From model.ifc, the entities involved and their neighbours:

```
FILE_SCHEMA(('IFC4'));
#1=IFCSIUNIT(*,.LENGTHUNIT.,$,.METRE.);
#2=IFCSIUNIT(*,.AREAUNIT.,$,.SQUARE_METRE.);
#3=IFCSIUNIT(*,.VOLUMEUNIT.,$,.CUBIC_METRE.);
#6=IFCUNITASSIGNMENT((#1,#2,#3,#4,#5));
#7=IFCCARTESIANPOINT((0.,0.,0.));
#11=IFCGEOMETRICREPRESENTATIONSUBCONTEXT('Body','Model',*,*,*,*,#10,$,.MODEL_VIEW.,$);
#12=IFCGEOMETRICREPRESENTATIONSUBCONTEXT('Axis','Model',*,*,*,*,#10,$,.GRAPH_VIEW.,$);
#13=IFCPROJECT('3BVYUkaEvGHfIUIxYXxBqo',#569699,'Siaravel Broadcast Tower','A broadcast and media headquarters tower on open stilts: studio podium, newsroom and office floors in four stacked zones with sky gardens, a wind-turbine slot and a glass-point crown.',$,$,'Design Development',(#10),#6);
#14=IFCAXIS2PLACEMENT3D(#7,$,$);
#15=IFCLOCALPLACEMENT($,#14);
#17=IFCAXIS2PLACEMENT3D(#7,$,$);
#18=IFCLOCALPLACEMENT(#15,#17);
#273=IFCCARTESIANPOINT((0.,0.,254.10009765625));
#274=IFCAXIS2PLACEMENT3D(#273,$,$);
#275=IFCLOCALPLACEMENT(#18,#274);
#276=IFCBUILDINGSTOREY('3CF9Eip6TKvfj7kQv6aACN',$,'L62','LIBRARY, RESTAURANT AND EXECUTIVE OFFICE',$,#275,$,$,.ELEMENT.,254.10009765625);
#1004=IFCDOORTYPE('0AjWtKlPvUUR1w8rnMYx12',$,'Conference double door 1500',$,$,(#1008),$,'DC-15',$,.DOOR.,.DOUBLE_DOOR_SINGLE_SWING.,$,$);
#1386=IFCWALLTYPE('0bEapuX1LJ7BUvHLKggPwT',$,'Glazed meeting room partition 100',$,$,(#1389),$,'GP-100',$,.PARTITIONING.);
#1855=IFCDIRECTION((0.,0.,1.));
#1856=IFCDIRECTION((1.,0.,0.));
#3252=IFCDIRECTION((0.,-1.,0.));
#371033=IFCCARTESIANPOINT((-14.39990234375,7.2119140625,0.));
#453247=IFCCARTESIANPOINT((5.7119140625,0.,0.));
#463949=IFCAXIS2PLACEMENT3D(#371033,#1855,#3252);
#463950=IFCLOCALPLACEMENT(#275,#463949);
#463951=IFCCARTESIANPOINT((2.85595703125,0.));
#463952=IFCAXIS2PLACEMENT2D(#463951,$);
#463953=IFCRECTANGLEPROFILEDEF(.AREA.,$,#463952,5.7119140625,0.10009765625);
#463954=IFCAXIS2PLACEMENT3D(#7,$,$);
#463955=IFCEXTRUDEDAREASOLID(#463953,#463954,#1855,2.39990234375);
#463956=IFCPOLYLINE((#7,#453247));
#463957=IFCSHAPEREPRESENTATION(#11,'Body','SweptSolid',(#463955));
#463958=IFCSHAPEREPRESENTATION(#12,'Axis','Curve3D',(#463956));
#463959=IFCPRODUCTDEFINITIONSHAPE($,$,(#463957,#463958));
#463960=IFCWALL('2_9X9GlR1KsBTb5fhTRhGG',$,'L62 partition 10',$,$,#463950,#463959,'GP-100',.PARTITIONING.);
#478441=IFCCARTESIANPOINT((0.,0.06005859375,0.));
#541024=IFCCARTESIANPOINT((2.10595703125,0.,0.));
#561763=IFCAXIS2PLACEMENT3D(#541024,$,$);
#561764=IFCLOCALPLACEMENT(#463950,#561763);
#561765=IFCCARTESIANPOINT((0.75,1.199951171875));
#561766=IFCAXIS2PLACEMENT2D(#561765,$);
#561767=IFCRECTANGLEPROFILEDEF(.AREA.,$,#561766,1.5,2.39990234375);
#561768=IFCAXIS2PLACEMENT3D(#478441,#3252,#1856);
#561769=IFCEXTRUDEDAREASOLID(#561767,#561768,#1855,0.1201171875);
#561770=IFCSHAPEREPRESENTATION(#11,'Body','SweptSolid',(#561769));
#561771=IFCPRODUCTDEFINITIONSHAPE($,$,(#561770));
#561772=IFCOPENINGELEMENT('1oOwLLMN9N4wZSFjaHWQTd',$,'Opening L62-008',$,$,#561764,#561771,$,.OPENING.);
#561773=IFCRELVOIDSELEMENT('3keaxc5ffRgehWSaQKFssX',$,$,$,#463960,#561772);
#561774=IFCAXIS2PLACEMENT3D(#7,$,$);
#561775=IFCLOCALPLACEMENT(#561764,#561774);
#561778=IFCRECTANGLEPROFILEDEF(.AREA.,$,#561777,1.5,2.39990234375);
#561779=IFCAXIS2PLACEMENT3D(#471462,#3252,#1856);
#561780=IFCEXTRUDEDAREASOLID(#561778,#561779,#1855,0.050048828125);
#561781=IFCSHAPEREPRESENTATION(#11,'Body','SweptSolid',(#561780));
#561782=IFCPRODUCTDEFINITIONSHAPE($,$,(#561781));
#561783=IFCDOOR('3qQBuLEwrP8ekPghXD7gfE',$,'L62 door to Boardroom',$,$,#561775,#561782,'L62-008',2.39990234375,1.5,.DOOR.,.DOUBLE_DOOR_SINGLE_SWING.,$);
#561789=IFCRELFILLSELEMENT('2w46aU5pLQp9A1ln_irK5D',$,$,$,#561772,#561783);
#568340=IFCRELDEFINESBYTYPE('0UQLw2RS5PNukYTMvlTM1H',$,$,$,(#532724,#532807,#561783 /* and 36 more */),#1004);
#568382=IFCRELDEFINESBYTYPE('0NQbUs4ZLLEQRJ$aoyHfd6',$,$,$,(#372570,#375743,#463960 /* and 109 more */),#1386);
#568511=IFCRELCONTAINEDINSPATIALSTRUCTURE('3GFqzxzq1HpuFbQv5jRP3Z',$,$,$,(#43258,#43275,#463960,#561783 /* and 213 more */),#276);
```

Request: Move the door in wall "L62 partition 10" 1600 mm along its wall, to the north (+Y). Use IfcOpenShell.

```python
import ifcopenshell
import ifcopenshell.api.geometry
import ifcopenshell.util.placement
import ifcopenshell.util.unit

model = ifcopenshell.open("model.ifc")
unit_scale = ifcopenshell.util.unit.calculate_unit_scale(model)

door = model.by_id(561783)
opening = door.FillsVoids[0].RelatingOpeningElement
wall = opening.VoidsElements[0].RelatingBuildingElement

wall_matrix = ifcopenshell.util.placement.get_local_placement(wall.ObjectPlacement)
shift = wall_matrix[:3, 0] * -1.6 / unit_scale
before = ifcopenshell.util.placement.get_local_placement(door.ObjectPlacement)[:3, 3].copy()

# The door is placed relative to its opening, so it follows when the opening moves.
matrix = ifcopenshell.util.placement.get_local_placement(opening.ObjectPlacement)
matrix[:3, 3] += shift
ifcopenshell.api.geometry.edit_object_placement(
    model, product=opening, matrix=matrix, is_si=False, should_transform_children=True
)

after = ifcopenshell.util.placement.get_local_placement(door.ObjectPlacement)[:3, 3]
print("door moved by", (after - before).round(3) + 0.0)

model.write("model_edited.ifc")
```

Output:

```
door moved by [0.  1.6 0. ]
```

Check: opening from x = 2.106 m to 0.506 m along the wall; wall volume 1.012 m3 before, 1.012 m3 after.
